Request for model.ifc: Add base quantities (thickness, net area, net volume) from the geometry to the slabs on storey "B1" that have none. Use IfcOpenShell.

First a look at what the model holds.

```python
import ifcopenshell
import ifcopenshell.util.element
import ifcopenshell.util.unit

model = ifcopenshell.open("model.ifc")
print(model.schema)
for unit_type in ("LENGTHUNIT", "AREAUNIT", "VOLUMEUNIT"):
    print(unit_type, ifcopenshell.util.unit.calculate_unit_scale(model, unit_type))
storey = next(s for s in model.by_type("IfcBuildingStorey") if s.Name == "B1")
slabs = [e for e in ifcopenshell.util.element.get_decomposition(storey) if e.is_a("IfcSlab")]
for e in sorted(slabs, key=lambda e: e.id()):
    print(e.id(), e.is_a(), e.Name, list(ifcopenshell.util.element.get_psets(e, qtos_only=True)), sep=" | ")
```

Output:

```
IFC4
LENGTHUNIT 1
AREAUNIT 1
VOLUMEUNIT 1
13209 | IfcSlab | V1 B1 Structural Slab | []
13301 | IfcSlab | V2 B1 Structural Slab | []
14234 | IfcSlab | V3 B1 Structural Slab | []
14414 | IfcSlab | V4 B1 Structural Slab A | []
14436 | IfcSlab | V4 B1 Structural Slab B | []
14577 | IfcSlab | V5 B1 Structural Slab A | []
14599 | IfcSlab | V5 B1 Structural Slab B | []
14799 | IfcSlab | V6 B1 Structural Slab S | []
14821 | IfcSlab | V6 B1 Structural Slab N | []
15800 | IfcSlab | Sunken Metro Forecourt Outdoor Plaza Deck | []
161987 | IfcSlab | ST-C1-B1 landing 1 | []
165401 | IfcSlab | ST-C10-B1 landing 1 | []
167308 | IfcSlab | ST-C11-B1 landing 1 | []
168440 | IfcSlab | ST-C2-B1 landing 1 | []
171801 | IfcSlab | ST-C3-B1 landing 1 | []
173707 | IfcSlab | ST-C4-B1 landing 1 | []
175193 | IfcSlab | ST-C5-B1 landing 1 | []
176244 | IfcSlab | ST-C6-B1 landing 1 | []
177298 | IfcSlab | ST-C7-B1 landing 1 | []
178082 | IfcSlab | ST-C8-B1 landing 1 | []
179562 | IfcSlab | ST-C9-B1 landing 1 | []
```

```python
import ifcopenshell
import ifcopenshell.api.pset
import ifcopenshell.geom
import ifcopenshell.util.element
import ifcopenshell.util.shape
import ifcopenshell.util.unit

model = ifcopenshell.open("model.ifc")
unit_scale = ifcopenshell.util.unit.calculate_unit_scale(model)
area_scale = ifcopenshell.util.unit.calculate_unit_scale(model, "AREAUNIT")
volume_scale = ifcopenshell.util.unit.calculate_unit_scale(model, "VOLUMEUNIT")
settings = ifcopenshell.geom.settings()

storey = next(s for s in model.by_type("IfcBuildingStorey") if s.Name == "B1")
slabs = [e for e in ifcopenshell.util.element.get_decomposition(storey) if e.is_a("IfcSlab")]

for e in sorted(slabs, key=lambda e: e.id()):
    if ifcopenshell.util.element.get_psets(e, qtos_only=True, should_inherit=False):
        continue
    # Geometry comes back in metres, in the element's own axes.
    shape = ifcopenshell.geom.create_shape(settings, e)
    values = {
        "Width": ifcopenshell.util.shape.get_z(shape.geometry) / unit_scale,
        "NetArea": ifcopenshell.util.shape.get_footprint_area(shape.geometry) / area_scale,
        "NetVolume": ifcopenshell.util.shape.get_volume(shape.geometry) / volume_scale,
    }
    qto = ifcopenshell.api.pset.add_qto(model, product=e, name="Qto_SlabBaseQuantities")
    ifcopenshell.api.pset.edit_qto(model, qto=qto, properties=values)
    print(e.id(), {k: round(v, 3) for k, v in values.items()})

model.write("model_v2.ifc")
```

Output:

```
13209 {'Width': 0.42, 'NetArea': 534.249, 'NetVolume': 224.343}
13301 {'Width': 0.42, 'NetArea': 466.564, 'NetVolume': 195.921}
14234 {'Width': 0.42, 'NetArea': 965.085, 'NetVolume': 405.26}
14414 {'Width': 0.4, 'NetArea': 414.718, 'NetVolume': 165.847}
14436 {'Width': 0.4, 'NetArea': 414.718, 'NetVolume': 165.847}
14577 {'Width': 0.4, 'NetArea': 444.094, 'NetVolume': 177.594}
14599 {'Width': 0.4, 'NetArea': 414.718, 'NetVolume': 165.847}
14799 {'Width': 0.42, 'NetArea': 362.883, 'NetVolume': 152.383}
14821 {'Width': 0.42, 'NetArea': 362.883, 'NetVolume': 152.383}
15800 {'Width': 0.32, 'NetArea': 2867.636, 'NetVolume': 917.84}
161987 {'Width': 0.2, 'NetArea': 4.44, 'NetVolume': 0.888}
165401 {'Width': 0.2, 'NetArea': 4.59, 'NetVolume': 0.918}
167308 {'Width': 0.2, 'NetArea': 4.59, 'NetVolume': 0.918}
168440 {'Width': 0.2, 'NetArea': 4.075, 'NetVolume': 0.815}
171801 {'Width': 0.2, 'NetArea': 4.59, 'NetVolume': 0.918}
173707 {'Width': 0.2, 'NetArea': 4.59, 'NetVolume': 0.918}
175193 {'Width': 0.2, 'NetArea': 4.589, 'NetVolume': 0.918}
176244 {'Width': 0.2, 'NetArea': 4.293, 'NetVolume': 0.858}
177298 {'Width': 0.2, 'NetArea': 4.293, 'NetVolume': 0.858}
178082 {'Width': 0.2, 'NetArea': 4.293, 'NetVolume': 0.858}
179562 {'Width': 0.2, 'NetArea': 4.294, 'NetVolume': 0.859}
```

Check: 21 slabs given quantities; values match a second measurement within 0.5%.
